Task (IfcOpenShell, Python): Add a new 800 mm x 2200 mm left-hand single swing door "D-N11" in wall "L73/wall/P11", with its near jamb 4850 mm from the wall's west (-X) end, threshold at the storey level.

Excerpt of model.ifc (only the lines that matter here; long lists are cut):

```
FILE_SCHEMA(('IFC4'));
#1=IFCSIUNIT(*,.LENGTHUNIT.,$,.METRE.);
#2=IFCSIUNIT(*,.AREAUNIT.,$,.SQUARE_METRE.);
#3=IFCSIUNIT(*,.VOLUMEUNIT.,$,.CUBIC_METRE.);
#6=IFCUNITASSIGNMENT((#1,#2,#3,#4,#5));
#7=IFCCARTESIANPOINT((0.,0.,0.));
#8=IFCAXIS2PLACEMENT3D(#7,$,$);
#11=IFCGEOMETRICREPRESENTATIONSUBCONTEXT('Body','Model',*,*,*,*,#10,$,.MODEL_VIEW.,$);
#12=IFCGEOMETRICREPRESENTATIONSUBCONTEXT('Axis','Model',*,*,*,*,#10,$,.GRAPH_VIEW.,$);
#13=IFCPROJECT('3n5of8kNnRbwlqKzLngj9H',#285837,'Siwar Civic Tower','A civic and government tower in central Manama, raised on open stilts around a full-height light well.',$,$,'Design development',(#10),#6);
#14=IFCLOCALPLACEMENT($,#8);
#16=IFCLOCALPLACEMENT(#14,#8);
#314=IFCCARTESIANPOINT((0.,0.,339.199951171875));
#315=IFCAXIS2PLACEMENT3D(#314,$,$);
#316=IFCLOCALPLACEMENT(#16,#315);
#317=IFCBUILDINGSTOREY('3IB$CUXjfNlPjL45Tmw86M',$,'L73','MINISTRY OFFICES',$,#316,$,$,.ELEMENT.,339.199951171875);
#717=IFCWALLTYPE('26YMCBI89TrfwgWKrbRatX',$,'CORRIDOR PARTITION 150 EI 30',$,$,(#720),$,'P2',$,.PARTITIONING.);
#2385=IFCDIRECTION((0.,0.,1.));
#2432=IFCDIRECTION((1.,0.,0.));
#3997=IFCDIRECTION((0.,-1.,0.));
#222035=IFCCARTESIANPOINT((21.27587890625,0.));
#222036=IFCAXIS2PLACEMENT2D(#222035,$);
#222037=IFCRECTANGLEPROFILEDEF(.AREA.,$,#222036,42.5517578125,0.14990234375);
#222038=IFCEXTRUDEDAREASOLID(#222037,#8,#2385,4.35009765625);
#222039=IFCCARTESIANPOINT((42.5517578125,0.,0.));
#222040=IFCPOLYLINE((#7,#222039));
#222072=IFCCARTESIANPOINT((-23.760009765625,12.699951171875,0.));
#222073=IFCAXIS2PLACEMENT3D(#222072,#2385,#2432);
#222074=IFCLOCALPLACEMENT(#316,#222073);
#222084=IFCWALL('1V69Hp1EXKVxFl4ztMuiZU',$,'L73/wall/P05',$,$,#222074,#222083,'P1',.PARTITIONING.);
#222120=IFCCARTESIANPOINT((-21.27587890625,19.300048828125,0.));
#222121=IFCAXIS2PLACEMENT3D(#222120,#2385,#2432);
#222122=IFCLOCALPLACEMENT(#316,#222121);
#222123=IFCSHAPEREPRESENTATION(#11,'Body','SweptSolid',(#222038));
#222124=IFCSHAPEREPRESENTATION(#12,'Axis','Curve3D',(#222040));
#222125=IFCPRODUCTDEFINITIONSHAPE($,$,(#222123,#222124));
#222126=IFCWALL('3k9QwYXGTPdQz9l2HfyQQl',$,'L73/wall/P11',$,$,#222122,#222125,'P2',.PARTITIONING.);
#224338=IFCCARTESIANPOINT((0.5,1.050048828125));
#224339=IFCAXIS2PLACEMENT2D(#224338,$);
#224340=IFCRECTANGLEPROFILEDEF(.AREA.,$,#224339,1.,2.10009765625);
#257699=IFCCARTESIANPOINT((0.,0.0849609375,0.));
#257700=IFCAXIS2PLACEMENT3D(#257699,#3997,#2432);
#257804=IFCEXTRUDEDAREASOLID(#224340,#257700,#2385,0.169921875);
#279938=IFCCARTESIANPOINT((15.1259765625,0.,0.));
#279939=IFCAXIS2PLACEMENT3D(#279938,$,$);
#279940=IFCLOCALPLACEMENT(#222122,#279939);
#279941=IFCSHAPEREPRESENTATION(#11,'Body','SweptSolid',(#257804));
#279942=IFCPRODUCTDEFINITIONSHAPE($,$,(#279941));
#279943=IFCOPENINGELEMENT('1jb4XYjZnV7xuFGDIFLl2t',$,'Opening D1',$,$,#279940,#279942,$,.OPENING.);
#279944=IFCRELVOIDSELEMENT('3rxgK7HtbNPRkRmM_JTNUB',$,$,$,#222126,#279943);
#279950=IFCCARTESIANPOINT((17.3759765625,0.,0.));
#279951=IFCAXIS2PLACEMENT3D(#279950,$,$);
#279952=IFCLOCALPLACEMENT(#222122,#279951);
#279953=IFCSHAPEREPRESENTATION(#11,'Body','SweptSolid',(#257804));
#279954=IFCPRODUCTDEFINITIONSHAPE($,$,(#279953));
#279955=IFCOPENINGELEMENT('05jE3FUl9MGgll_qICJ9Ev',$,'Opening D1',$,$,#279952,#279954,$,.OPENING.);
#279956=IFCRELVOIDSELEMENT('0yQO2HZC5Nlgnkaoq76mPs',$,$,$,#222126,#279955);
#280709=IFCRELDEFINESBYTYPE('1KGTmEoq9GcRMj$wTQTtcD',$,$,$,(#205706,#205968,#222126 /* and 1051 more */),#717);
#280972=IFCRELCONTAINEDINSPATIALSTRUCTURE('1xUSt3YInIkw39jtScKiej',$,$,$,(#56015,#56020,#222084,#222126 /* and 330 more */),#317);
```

```python
import numpy as np
import ifcopenshell
import ifcopenshell.api.feature
import ifcopenshell.api.geometry
import ifcopenshell.api.root
import ifcopenshell.api.spatial
import ifcopenshell.geom
import ifcopenshell.util.element
import ifcopenshell.util.placement
import ifcopenshell.util.representation
import ifcopenshell.util.shape
import ifcopenshell.util.unit

model = ifcopenshell.open("model.ifc")
unit_scale = ifcopenshell.util.unit.calculate_unit_scale(model)
settings = ifcopenshell.geom.settings()


def volume(element):
    """Net volume in cubic metres, openings subtracted."""
    shape = ifcopenshell.geom.create_shape(settings, element)
    return ifcopenshell.util.shape.get_volume(shape.geometry)


wall = model.by_id(222126)
storey = ifcopenshell.util.element.get_container(wall, ifc_class="IfcBuildingStorey")
context = ifcopenshell.util.representation.get_context(model, "Model", "Body", "MODEL_VIEW")
before = volume(wall)

width, height, from_end, sill = 0.8, 2.2, 4.85, 0.0  # metres

# The wall runs along its own X axis, and the end named is its -X end.
wall_shape = ifcopenshell.geom.create_shape(settings, wall)
x, y, z = ifcopenshell.util.shape.get_vertices(wall_shape.geometry).T
start = x.min() + from_end
face, thickness = float(y.min()), float(y.max() - y.min())
wall_matrix = ifcopenshell.util.placement.get_local_placement(wall.ObjectPlacement)
level = ifcopenshell.util.placement.get_local_placement(storey.ObjectPlacement)[2, 3]


def in_wall(x, y):
    """Placement at x, y metres in the wall's axes, at sill height."""
    matrix = wall_matrix.copy()
    matrix[:, 3] = wall_matrix @ np.array([x / unit_scale, y / unit_scale, 0.0, 1.0])
    matrix[2, 3] = level + sill / unit_scale
    return matrix


# Opening: a box that overshoots both wall faces by 50 mm.
opening = ifcopenshell.api.root.create_entity(model, ifc_class="IfcOpeningElement", predefined_type="OPENING")
box = ifcopenshell.api.geometry.add_wall_representation(
    model, context=context, length=width, height=height, thickness=thickness + 0.1
)
ifcopenshell.api.geometry.assign_representation(model, product=opening, representation=box)
ifcopenshell.api.geometry.edit_object_placement(model, product=opening, matrix=in_wall(start, face - 0.05), is_si=False)
ifcopenshell.api.feature.add_feature(model, feature=opening, element=wall)

door = ifcopenshell.api.root.create_entity(model, ifc_class="IfcDoor", name="D-N11", predefined_type="DOOR")
door.OverallWidth, door.OverallHeight = width / unit_scale, height / unit_scale
door.OperationType = "SINGLE_SWING_LEFT"
body = ifcopenshell.api.geometry.add_door_representation(
    model,
    context=context,
    overall_width=door.OverallWidth,
    overall_height=door.OverallHeight,
    operation_type="SINGLE_SWING_LEFT",
    lining_properties={"LiningDepth": thickness / unit_scale, "ThresholdDepth": thickness / unit_scale},
)
ifcopenshell.api.geometry.assign_representation(model, product=door, representation=body)
ifcopenshell.api.spatial.assign_container(model, products=[door], relating_structure=storey)
ifcopenshell.api.feature.add_filling(model, opening=opening, element=door)

# The lining spans the wall, so the door starts at the wall face.
ifcopenshell.api.geometry.edit_object_placement(model, product=door, matrix=in_wall(start, face), is_si=False)

after = volume(wall)

print(f"wall volume {before:.3f} -> {after:.3f} m3")

model.write("model-out.ifc")
```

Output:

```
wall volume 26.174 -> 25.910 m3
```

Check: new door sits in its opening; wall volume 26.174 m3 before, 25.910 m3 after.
